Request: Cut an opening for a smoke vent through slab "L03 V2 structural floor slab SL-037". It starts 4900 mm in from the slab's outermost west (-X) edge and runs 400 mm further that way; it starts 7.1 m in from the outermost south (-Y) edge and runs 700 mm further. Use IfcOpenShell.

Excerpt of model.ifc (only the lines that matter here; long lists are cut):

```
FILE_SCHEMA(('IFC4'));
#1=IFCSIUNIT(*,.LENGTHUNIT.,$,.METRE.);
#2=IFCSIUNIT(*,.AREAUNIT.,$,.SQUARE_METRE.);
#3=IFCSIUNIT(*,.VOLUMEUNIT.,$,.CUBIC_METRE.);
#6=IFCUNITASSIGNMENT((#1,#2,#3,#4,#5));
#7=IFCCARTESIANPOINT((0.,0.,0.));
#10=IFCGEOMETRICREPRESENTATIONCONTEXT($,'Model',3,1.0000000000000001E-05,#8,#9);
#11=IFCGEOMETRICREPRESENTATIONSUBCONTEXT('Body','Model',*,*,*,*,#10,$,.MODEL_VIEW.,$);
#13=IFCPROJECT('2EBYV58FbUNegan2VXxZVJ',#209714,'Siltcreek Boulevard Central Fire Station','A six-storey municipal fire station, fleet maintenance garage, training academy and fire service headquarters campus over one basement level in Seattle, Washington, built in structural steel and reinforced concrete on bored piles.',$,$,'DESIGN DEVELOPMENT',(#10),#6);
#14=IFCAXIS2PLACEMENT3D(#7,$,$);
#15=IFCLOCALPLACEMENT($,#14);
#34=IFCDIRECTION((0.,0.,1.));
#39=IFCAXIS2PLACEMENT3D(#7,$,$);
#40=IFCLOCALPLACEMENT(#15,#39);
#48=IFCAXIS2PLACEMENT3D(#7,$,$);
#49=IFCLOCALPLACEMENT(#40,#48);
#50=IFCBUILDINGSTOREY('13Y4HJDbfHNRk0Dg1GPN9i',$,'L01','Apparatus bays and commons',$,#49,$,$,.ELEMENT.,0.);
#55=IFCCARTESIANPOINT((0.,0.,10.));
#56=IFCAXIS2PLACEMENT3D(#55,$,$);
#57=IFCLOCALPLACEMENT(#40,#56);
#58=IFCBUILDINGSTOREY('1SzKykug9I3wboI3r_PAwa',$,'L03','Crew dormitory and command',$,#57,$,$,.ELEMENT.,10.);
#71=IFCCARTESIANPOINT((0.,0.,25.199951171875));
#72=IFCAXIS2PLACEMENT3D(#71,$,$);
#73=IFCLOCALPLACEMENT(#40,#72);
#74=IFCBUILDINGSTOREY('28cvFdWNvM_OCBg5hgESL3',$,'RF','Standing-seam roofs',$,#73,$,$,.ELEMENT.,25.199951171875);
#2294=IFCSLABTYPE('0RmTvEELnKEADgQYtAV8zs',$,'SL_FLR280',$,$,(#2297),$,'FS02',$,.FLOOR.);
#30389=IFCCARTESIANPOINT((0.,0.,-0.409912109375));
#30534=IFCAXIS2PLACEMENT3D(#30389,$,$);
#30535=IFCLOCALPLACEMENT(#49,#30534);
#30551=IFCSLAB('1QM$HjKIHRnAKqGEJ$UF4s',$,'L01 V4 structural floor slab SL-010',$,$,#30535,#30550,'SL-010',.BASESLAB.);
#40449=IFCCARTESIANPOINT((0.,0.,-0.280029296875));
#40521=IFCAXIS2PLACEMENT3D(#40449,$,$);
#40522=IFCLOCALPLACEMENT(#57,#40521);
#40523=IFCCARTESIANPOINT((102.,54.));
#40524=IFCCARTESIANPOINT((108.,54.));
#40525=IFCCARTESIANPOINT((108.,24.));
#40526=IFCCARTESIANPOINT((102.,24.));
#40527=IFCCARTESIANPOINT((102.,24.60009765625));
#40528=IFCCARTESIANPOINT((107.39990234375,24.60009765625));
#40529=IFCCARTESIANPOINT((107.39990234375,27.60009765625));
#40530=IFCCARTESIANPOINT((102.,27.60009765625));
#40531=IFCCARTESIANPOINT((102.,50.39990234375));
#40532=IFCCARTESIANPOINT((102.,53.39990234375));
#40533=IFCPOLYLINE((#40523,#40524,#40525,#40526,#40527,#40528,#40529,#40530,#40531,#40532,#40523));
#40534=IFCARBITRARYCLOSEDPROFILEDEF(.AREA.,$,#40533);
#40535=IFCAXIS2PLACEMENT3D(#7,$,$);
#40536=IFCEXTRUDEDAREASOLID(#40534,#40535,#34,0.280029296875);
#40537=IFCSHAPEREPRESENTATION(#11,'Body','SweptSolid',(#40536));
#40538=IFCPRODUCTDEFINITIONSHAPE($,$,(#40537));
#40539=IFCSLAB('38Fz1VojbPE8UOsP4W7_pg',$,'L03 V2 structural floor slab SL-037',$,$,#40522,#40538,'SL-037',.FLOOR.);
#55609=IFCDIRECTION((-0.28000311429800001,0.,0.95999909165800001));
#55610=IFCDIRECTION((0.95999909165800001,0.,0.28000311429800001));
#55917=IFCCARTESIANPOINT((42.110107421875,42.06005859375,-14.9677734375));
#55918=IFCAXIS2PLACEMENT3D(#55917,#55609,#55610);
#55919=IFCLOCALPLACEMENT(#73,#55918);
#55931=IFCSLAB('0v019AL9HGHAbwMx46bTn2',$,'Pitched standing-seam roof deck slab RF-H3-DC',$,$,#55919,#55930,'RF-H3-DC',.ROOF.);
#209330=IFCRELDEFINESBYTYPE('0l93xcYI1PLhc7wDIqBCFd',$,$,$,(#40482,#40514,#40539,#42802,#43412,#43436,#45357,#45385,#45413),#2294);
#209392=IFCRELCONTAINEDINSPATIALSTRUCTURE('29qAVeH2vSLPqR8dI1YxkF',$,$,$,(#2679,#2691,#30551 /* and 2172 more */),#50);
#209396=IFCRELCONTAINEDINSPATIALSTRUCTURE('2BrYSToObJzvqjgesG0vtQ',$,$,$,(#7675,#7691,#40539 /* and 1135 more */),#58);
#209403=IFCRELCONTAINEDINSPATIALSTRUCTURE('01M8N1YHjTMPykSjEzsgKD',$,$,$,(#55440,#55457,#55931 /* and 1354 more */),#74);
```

```python
import numpy as np
import ifcopenshell
import ifcopenshell.api.feature
import ifcopenshell.api.geometry
import ifcopenshell.api.root
import ifcopenshell.geom
import ifcopenshell.util.placement
import ifcopenshell.util.representation
import ifcopenshell.util.shape
import ifcopenshell.util.unit

model = ifcopenshell.open("model.ifc")
unit_scale = ifcopenshell.util.unit.calculate_unit_scale(model)
settings = ifcopenshell.geom.settings()


def volume(element):
    """Net volume in cubic metres, openings subtracted."""
    shape = ifcopenshell.geom.create_shape(settings, element)
    return ifcopenshell.util.shape.get_volume(shape.geometry)


slab = model.by_guid("38Fz1VojbPE8UOsP4W7_pg")
before = volume(slab)

# Extent in the slab's own axes, in metres. The edges named are its -X and -Y sides.
slab_shape = ifcopenshell.geom.create_shape(settings, slab)
vertices = ifcopenshell.util.shape.get_vertices(slab_shape.geometry)
x_min, y_min, bottom = vertices.min(axis=0)
top = vertices[:, 2].max()

opening = ifcopenshell.api.root.create_entity(model, ifc_class="IfcOpeningElement", name="Smoke vent opening", predefined_type="OPENING")
context = ifcopenshell.util.representation.get_context(model, "Model", "Body", "MODEL_VIEW")
width, depth = 0.4, 0.7
outline = [(0.0, 0.0), (width, 0.0), (width, depth), (0.0, depth), (0.0, 0.0)]
# Overshoot both faces by 50 mm so the cut is clean.
shape = ifcopenshell.api.geometry.add_slab_representation(
    model, context=context, depth=top - bottom + 0.1, polyline=outline
)
ifcopenshell.api.geometry.assign_representation(model, product=opening, representation=shape)

matrix = ifcopenshell.util.placement.get_local_placement(slab.ObjectPlacement)
matrix[:, 3] = matrix @ np.append(np.array([x_min + 4.9, y_min + 7.1, bottom - 0.05]) / unit_scale, 1.0)
ifcopenshell.api.geometry.edit_object_placement(model, product=opening, matrix=matrix, is_si=False)
ifcopenshell.api.feature.add_feature(model, feature=opening, element=slab)

after = volume(slab)

print(f"slab volume {before:.3f} -> {after:.3f} m3")

model.write("model_updated.ifc")
```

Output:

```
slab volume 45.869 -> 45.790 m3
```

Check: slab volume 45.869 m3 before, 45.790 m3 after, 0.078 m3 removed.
